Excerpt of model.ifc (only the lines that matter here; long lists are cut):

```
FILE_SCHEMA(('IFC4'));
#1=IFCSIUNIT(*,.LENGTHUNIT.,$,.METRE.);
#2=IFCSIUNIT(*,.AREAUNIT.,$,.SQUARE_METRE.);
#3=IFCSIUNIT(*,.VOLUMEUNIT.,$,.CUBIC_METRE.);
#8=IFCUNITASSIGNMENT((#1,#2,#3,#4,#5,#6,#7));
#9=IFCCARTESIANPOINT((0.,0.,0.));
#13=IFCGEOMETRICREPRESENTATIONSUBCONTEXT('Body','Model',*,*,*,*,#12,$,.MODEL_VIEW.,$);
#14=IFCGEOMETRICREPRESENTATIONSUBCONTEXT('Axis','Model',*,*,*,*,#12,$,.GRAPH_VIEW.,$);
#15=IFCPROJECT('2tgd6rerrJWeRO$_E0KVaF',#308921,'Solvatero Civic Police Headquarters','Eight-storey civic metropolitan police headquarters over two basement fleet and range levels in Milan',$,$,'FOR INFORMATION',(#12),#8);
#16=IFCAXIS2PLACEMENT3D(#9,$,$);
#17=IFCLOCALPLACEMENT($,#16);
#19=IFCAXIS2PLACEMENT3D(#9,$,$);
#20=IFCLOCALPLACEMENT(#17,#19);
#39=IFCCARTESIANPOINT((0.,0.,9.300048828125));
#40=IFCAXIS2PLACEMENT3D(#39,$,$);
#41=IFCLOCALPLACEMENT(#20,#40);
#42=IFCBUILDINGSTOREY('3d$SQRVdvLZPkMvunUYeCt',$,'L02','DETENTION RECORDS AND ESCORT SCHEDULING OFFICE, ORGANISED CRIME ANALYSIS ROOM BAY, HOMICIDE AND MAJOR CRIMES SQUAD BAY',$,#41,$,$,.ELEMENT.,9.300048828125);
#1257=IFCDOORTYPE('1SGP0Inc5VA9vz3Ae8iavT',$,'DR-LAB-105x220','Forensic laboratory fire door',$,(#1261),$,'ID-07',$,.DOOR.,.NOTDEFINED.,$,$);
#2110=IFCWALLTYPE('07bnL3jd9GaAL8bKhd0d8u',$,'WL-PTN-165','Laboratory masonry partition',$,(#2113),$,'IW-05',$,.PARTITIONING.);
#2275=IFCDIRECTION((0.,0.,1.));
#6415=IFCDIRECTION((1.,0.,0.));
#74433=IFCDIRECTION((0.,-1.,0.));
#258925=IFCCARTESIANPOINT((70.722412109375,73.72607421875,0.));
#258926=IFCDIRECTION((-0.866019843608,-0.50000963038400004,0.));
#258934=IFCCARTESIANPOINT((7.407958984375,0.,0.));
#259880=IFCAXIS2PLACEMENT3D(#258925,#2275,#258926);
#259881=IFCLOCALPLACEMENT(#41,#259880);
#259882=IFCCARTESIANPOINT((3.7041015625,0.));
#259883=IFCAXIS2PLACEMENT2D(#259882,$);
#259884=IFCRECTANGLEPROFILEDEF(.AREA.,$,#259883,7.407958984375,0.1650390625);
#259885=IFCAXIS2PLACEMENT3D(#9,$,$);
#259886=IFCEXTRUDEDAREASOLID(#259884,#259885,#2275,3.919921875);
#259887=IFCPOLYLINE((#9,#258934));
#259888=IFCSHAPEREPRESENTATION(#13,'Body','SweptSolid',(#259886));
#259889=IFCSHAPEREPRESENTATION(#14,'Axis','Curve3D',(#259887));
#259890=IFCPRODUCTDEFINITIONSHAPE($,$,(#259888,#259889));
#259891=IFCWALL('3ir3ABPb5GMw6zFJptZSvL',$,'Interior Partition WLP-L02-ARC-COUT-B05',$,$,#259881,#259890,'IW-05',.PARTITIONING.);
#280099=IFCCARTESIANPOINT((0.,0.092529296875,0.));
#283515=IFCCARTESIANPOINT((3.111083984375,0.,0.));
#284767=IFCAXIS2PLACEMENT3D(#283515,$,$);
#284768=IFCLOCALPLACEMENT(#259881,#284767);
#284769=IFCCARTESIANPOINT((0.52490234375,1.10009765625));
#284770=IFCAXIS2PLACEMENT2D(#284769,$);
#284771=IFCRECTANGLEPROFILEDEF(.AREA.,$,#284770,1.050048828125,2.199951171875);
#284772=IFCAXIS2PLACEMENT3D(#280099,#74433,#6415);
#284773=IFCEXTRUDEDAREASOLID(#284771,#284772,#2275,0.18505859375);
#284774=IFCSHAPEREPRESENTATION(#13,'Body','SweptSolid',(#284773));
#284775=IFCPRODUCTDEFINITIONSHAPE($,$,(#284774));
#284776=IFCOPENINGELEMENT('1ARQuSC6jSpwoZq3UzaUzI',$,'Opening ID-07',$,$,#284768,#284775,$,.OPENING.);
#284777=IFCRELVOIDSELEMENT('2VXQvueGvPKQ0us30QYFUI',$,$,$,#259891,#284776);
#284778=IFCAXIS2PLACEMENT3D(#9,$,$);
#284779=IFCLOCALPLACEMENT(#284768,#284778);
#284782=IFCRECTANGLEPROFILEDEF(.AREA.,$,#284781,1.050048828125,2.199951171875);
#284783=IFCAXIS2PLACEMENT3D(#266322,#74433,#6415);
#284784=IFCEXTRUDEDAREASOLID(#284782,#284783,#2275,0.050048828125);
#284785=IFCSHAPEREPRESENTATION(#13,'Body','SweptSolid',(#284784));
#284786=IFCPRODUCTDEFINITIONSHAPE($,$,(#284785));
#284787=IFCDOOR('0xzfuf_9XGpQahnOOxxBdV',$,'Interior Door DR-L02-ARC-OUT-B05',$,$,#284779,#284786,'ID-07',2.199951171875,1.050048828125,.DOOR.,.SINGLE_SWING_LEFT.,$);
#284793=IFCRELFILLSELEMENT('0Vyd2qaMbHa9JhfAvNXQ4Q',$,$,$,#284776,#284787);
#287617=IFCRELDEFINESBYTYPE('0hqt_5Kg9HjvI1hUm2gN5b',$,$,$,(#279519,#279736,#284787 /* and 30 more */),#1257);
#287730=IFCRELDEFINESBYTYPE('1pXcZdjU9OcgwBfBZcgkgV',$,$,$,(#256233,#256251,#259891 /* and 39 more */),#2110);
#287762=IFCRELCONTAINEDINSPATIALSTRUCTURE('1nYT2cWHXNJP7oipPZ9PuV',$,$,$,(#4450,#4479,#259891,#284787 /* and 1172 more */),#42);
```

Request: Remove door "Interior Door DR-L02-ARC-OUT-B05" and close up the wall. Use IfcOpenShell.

```python
import ifcopenshell
import ifcopenshell.api.feature
import ifcopenshell.api.root
import ifcopenshell.geom
import ifcopenshell.util.shape

model = ifcopenshell.open("model.ifc")
settings = ifcopenshell.geom.settings()


def volume(element):
    """Net volume in cubic metres, openings subtracted."""
    shape = ifcopenshell.geom.create_shape(settings, element)
    return ifcopenshell.util.shape.get_volume(shape.geometry)


door = model.by_guid("0xzfuf_9XGpQahnOOxxBdV")
opening = door.FillsVoids[0].RelatingOpeningElement
wall = opening.VoidsElements[0].RelatingBuildingElement
before = volume(wall)

ifcopenshell.api.root.remove_product(model, product=door)
ifcopenshell.api.feature.remove_feature(model, feature=opening)

after = volume(wall)

print(f"wall volume {before:.3f} -> {after:.3f} m3")

model.write("model-out.ifc")
```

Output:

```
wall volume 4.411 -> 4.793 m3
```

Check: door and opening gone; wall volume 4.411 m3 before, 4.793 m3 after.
